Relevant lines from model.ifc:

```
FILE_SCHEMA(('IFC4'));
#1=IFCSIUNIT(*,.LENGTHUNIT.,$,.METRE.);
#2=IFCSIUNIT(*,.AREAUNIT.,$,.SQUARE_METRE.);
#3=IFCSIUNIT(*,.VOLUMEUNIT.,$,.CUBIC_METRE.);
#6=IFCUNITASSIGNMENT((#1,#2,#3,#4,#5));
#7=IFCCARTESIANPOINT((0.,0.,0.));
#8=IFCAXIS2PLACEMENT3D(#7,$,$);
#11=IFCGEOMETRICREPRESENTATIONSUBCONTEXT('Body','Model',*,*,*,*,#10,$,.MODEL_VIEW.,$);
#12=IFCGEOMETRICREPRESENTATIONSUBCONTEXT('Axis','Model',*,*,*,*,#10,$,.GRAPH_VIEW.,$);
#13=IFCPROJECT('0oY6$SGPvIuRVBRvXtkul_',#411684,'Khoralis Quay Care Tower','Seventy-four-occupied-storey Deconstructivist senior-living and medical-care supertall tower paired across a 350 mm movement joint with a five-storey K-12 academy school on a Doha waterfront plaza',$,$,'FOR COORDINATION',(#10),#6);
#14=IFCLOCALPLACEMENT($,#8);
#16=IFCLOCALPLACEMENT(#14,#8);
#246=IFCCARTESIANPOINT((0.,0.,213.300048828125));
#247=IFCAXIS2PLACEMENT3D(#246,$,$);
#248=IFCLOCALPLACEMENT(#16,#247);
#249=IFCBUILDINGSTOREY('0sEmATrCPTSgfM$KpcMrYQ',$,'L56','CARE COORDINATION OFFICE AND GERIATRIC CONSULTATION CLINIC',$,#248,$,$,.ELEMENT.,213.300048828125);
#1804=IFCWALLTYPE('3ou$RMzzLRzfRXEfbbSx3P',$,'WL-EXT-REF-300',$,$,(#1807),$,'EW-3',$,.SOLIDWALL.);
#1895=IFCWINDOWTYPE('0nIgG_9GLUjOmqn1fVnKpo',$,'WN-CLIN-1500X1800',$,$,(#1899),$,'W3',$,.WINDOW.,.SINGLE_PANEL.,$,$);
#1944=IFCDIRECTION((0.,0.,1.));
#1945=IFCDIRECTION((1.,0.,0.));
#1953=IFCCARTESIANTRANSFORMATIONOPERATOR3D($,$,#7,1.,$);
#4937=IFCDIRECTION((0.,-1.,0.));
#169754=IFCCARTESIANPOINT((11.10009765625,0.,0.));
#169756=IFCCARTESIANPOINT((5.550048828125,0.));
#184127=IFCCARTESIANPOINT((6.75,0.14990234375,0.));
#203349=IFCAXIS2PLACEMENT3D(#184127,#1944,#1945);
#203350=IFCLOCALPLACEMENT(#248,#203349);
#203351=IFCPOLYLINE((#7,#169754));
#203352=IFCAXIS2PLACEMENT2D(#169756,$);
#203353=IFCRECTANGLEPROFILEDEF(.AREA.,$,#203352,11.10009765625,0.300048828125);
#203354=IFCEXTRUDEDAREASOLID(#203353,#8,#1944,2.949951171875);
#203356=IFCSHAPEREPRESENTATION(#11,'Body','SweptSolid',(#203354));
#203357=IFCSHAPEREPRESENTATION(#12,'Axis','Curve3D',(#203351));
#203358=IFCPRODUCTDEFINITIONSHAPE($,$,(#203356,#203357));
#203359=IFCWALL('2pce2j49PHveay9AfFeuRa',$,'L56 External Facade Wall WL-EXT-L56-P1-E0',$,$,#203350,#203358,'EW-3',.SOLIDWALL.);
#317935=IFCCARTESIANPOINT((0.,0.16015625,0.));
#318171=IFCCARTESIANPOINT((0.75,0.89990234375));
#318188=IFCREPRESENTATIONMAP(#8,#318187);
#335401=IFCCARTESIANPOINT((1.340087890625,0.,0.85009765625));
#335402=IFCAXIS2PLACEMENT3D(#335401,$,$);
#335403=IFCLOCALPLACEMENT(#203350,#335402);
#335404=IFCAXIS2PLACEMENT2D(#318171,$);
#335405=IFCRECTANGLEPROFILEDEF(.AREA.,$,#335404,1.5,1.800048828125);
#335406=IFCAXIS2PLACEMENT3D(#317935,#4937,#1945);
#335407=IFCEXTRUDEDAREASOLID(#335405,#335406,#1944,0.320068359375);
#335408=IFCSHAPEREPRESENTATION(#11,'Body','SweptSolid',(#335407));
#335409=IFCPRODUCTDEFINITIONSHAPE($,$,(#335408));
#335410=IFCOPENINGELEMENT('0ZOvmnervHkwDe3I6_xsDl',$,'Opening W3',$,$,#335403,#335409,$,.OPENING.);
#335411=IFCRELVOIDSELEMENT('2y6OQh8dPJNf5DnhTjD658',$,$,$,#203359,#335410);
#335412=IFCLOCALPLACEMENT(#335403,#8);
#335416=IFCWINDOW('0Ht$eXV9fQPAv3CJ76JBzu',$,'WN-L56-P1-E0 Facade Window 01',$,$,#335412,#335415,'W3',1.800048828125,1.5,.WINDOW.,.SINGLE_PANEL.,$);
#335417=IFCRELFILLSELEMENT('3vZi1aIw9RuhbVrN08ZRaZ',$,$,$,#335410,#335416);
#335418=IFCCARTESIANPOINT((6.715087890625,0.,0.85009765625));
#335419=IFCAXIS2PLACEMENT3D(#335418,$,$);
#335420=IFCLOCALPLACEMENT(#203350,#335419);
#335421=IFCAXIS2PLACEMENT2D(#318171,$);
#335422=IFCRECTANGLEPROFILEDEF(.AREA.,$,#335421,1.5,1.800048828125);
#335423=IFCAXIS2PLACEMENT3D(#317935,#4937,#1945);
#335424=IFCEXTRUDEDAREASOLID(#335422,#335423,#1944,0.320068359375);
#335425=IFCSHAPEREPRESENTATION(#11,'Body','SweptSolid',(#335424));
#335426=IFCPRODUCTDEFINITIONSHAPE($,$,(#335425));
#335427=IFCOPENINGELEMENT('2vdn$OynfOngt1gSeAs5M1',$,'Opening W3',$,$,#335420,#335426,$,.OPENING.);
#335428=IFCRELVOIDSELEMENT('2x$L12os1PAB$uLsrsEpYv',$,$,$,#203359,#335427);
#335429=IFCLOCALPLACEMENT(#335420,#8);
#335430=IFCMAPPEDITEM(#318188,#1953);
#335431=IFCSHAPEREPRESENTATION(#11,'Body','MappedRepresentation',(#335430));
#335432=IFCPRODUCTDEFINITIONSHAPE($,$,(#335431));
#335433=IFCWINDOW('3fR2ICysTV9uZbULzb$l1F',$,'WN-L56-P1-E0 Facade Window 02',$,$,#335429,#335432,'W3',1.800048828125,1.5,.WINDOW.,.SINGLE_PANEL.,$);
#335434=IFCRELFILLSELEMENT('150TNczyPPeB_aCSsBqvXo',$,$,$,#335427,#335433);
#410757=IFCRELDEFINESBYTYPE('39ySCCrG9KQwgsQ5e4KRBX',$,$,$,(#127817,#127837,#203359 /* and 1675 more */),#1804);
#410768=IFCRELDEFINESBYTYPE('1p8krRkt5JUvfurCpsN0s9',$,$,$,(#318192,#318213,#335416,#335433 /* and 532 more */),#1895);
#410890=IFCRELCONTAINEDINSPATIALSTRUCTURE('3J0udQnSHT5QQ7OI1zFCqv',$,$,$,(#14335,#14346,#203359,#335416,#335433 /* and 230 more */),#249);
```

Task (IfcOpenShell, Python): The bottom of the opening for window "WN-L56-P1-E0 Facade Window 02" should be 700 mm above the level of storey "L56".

```python
import numpy as np
import ifcopenshell
import ifcopenshell.api.geometry
import ifcopenshell.geom
import ifcopenshell.util.element
import ifcopenshell.util.placement
import ifcopenshell.util.shape
import ifcopenshell.util.unit

model = ifcopenshell.open("model.ifc")
unit_scale = ifcopenshell.util.unit.calculate_unit_scale(model)

window = model.by_id(335433)
opening = window.FillsVoids[0].RelatingOpeningElement
storey = ifcopenshell.util.element.get_container(window, ifc_class="IfcBuildingStorey")
level = ifcopenshell.util.placement.get_local_placement(storey.ObjectPlacement)[2, 3]

# The opening's origin need not be at the sill, so measure its lowest point.
shape = ifcopenshell.geom.create_shape(ifcopenshell.geom.settings(), opening)
bottom = ifcopenshell.util.shape.get_shape_bottom_elevation(shape, shape.geometry) / unit_scale
dz = level + 0.7 - bottom

shift = np.array([0.0, 0.0, dz])
# The window is placed relative to its opening, so it follows when the opening moves.
matrix = ifcopenshell.util.placement.get_local_placement(opening.ObjectPlacement)
matrix[:3, 3] += shift
ifcopenshell.api.geometry.edit_object_placement(
    model, product=opening, matrix=matrix, is_si=False, should_transform_children=True
)

print(f"moved by {dz * unit_scale:+.3f} m")

model.write("model-out.ifc")
```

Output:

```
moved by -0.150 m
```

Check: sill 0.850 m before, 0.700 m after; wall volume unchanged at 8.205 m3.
